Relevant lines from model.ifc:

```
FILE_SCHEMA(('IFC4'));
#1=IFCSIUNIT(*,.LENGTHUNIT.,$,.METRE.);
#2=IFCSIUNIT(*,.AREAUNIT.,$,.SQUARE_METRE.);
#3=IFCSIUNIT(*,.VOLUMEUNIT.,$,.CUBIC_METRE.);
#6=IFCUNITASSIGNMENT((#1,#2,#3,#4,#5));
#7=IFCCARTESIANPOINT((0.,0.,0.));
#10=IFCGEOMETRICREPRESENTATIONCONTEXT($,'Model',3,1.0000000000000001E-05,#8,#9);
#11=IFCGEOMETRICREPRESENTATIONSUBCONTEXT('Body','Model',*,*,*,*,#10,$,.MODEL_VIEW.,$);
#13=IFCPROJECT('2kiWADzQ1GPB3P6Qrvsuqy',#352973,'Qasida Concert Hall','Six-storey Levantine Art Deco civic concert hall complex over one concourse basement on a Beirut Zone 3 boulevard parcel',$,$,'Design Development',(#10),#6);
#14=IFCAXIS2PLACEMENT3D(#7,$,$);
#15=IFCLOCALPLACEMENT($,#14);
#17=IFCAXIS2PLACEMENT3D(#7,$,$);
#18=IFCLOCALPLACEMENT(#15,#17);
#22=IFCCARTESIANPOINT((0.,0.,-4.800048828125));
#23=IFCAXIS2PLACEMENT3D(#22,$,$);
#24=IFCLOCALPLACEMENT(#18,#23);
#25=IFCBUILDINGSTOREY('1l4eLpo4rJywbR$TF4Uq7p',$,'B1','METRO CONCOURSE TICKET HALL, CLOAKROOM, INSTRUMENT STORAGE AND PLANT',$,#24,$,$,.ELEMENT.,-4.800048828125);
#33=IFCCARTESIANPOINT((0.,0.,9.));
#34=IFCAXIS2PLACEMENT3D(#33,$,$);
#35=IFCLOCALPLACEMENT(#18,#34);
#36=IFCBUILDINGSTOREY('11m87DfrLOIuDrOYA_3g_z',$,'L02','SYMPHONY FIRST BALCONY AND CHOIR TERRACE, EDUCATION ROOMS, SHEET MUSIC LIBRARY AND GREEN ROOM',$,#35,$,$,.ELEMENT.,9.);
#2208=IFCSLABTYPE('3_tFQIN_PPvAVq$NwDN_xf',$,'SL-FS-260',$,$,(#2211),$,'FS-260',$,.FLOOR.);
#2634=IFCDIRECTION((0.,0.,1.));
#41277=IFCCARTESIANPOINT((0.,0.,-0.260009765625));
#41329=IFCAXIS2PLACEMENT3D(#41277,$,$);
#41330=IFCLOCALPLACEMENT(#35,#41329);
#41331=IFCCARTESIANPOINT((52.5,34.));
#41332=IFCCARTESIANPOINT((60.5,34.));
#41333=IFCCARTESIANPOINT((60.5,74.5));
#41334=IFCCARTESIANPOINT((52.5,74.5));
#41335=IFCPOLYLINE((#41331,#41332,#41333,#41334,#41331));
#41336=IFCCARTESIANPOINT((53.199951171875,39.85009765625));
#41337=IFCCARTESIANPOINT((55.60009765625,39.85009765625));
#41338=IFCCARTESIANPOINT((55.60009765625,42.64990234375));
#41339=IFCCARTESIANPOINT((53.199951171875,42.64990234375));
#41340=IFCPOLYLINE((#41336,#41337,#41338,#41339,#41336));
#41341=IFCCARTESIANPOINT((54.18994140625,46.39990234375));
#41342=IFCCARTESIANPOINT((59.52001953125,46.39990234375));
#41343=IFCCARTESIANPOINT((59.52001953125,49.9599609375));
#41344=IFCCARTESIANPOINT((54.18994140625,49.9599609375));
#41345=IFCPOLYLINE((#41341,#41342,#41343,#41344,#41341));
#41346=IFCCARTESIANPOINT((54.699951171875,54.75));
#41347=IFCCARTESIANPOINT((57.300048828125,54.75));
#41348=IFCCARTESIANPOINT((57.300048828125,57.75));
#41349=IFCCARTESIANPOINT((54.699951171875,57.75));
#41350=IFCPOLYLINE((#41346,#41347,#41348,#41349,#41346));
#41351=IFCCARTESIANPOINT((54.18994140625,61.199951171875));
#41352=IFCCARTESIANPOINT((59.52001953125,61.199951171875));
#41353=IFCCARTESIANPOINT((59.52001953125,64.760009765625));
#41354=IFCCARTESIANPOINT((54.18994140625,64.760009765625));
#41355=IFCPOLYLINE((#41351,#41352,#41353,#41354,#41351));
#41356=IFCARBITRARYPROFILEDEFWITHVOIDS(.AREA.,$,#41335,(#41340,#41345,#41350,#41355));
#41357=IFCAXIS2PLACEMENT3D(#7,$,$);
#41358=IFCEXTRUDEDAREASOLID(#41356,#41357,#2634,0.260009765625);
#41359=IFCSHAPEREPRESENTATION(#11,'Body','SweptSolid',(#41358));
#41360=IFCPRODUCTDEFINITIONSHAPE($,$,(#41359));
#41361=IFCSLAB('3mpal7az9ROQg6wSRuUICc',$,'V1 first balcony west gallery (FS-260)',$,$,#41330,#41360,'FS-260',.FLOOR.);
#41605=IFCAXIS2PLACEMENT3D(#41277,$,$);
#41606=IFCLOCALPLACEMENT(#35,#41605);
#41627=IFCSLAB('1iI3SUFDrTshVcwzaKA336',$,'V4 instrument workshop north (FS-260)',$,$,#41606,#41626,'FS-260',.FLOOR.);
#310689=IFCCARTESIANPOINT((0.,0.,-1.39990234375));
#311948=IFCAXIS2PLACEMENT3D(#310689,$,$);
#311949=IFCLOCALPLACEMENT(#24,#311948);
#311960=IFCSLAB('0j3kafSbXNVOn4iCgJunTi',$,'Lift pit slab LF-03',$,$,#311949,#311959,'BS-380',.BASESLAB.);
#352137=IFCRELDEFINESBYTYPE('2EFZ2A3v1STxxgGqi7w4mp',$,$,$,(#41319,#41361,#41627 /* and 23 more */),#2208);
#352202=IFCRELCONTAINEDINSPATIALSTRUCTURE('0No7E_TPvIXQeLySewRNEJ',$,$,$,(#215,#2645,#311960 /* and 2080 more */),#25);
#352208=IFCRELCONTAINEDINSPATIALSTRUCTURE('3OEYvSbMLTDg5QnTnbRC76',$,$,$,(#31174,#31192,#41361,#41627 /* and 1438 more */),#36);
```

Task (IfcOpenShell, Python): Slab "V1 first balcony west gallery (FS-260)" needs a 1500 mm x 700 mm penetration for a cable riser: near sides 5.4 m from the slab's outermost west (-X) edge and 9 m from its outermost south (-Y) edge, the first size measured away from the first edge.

```python
import numpy as np
import ifcopenshell
import ifcopenshell.api.feature
import ifcopenshell.api.geometry
import ifcopenshell.api.root
import ifcopenshell.geom
import ifcopenshell.util.placement
import ifcopenshell.util.representation
import ifcopenshell.util.shape
import ifcopenshell.util.unit

model = ifcopenshell.open("model.ifc")
unit_scale = ifcopenshell.util.unit.calculate_unit_scale(model)
settings = ifcopenshell.geom.settings()


def volume(element):
    """Net volume in cubic metres, openings subtracted."""
    shape = ifcopenshell.geom.create_shape(settings, element)
    return ifcopenshell.util.shape.get_volume(shape.geometry)


slab = model.by_guid("3mpal7az9ROQg6wSRuUICc")
before = volume(slab)

# Extent in the slab's own axes, in metres. The edges named are its -X and -Y sides.
slab_shape = ifcopenshell.geom.create_shape(settings, slab)
vertices = ifcopenshell.util.shape.get_vertices(slab_shape.geometry)
x_min, y_min, bottom = vertices.min(axis=0)
top = vertices[:, 2].max()

opening = ifcopenshell.api.root.create_entity(model, ifc_class="IfcOpeningElement", name="Cable riser opening", predefined_type="OPENING")
context = ifcopenshell.util.representation.get_context(model, "Model", "Body", "MODEL_VIEW")
width, depth = 1.5, 0.7
outline = [(0.0, 0.0), (width, 0.0), (width, depth), (0.0, depth), (0.0, 0.0)]
# Overshoot both faces by 50 mm so the cut is clean.
shape = ifcopenshell.api.geometry.add_slab_representation(
    model, context=context, depth=top - bottom + 0.1, polyline=outline
)
ifcopenshell.api.geometry.assign_representation(model, product=opening, representation=shape)

matrix = ifcopenshell.util.placement.get_local_placement(slab.ObjectPlacement)
matrix[:, 3] = matrix @ np.append(np.array([x_min + 5.4, y_min + 9, bottom - 0.05]) / unit_scale, 1.0)
ifcopenshell.api.geometry.edit_object_placement(model, product=opening, matrix=matrix, is_si=False)
ifcopenshell.api.feature.add_feature(model, feature=opening, element=slab)

after = volume(slab)

print(f"slab volume {before:.3f} -> {after:.3f} m3")

model.write("model_updated.ifc")
```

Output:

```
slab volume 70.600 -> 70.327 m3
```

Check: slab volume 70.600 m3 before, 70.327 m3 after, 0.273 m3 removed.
